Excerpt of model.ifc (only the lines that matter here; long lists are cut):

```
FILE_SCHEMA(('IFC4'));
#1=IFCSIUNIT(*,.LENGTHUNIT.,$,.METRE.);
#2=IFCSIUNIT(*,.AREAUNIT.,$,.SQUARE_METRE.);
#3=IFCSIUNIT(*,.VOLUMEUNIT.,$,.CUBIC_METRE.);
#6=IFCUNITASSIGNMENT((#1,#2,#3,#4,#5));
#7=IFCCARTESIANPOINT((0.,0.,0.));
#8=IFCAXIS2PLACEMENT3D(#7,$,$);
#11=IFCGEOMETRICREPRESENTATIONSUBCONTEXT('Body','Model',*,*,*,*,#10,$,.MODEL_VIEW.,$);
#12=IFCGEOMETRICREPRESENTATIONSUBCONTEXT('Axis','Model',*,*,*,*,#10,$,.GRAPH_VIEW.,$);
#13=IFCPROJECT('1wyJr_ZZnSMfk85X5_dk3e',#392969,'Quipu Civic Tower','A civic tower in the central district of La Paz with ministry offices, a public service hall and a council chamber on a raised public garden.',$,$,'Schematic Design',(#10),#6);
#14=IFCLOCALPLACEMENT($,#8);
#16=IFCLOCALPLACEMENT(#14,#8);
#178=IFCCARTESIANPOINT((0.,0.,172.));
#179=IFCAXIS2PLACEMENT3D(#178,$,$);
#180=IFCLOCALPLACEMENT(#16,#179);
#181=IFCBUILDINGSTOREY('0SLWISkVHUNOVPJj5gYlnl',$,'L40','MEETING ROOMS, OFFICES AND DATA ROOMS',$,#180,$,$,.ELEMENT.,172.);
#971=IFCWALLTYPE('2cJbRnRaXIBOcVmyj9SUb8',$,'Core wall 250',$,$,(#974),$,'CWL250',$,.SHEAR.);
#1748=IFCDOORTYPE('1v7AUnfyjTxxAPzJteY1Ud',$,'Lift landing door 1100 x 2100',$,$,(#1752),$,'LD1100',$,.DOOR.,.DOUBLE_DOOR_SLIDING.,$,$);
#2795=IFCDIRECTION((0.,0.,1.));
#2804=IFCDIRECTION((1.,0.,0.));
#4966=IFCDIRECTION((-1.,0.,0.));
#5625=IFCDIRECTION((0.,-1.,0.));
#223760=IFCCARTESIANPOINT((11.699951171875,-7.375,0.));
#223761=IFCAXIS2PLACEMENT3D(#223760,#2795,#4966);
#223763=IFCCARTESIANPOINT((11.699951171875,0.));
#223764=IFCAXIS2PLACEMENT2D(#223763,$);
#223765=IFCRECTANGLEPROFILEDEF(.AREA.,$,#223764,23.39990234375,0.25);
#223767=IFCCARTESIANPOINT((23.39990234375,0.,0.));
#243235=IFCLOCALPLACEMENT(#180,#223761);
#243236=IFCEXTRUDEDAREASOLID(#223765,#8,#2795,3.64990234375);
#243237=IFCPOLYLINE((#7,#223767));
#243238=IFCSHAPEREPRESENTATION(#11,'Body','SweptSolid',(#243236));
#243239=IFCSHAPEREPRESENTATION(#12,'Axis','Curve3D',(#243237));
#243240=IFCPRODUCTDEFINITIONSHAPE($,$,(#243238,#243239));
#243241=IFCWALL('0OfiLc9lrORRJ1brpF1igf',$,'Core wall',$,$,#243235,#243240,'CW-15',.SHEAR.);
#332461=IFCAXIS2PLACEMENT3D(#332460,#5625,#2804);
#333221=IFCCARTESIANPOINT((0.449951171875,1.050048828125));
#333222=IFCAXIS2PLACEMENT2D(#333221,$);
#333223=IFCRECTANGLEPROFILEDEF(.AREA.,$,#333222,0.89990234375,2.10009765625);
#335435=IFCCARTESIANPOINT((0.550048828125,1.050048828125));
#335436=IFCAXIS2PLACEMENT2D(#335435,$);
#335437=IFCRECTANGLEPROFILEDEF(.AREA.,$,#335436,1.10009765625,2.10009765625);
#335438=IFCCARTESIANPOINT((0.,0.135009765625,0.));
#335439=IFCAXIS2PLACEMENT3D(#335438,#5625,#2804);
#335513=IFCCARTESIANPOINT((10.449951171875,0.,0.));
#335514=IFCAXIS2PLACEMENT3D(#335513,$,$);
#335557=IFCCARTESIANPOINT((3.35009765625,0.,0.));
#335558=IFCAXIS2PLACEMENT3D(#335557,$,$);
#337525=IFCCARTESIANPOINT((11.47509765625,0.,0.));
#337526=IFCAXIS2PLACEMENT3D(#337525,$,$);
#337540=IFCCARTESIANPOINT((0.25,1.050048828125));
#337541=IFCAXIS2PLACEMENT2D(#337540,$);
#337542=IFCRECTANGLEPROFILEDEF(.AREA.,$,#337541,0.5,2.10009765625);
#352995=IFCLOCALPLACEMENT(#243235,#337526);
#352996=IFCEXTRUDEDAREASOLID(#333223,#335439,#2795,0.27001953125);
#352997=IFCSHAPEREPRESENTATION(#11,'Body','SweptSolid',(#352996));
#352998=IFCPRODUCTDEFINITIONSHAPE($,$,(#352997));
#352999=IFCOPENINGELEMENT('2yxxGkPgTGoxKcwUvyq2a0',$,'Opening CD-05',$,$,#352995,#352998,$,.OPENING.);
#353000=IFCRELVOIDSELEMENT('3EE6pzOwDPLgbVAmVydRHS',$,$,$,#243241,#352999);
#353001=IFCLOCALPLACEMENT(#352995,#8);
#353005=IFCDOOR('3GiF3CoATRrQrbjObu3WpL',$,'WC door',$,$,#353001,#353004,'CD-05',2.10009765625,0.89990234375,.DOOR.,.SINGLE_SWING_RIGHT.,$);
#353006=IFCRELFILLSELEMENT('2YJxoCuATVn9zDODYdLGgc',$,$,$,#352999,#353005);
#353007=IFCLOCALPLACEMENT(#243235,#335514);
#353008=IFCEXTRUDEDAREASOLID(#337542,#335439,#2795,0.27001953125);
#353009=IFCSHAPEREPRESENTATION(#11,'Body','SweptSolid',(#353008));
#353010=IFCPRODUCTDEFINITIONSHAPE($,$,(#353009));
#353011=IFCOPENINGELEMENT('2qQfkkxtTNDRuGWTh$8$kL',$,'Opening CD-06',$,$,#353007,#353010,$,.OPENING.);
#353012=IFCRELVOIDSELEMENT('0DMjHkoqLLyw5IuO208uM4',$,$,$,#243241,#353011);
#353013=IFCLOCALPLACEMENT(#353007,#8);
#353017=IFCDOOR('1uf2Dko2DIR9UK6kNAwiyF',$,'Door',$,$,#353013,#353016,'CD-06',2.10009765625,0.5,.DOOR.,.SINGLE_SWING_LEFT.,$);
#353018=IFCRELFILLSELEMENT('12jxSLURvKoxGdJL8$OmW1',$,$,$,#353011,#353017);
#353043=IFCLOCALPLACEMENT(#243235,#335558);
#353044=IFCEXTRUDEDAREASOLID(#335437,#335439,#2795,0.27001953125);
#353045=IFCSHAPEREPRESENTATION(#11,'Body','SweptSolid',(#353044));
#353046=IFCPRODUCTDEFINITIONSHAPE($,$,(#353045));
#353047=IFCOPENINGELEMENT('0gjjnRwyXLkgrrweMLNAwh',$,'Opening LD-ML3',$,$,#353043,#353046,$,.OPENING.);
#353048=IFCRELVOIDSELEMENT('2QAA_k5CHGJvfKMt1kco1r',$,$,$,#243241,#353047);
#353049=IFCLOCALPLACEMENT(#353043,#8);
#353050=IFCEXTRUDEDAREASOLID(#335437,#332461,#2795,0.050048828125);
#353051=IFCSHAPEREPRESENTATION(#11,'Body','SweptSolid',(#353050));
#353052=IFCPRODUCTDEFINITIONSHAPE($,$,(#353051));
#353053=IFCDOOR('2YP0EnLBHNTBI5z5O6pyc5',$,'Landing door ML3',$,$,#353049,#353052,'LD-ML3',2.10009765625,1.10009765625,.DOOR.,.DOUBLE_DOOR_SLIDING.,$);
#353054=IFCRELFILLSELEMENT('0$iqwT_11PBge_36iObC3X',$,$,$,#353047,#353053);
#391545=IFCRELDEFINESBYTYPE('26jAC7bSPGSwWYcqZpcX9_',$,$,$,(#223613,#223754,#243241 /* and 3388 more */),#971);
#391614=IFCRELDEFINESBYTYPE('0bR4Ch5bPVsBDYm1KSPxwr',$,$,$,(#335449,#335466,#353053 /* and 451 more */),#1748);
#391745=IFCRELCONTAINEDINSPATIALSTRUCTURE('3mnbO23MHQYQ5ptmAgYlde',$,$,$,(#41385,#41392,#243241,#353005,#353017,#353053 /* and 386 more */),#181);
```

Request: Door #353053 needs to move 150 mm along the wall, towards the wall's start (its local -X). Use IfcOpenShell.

```python
import ifcopenshell
import ifcopenshell.api.geometry
import ifcopenshell.util.placement
import ifcopenshell.util.unit

model = ifcopenshell.open("model.ifc")
unit_scale = ifcopenshell.util.unit.calculate_unit_scale(model)

door = model.by_guid("2YP0EnLBHNTBI5z5O6pyc5")
opening = door.FillsVoids[0].RelatingOpeningElement
wall = opening.VoidsElements[0].RelatingBuildingElement

wall_matrix = ifcopenshell.util.placement.get_local_placement(wall.ObjectPlacement)
shift = wall_matrix[:3, 0] * -0.15 / unit_scale
before = ifcopenshell.util.placement.get_local_placement(door.ObjectPlacement)[:3, 3].copy()

# The door is placed relative to its opening, so it follows when the opening moves.
matrix = ifcopenshell.util.placement.get_local_placement(opening.ObjectPlacement)
matrix[:3, 3] += shift
ifcopenshell.api.geometry.edit_object_placement(
    model, product=opening, matrix=matrix, is_si=False, should_transform_children=True
)

after = ifcopenshell.util.placement.get_local_placement(door.ObjectPlacement)[:3, 3]
print("door moved by", (after - before).round(3) + 0.0)

model.write("model_edited.ifc")
```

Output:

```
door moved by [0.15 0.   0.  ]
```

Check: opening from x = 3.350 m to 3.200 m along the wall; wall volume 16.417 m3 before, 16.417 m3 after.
